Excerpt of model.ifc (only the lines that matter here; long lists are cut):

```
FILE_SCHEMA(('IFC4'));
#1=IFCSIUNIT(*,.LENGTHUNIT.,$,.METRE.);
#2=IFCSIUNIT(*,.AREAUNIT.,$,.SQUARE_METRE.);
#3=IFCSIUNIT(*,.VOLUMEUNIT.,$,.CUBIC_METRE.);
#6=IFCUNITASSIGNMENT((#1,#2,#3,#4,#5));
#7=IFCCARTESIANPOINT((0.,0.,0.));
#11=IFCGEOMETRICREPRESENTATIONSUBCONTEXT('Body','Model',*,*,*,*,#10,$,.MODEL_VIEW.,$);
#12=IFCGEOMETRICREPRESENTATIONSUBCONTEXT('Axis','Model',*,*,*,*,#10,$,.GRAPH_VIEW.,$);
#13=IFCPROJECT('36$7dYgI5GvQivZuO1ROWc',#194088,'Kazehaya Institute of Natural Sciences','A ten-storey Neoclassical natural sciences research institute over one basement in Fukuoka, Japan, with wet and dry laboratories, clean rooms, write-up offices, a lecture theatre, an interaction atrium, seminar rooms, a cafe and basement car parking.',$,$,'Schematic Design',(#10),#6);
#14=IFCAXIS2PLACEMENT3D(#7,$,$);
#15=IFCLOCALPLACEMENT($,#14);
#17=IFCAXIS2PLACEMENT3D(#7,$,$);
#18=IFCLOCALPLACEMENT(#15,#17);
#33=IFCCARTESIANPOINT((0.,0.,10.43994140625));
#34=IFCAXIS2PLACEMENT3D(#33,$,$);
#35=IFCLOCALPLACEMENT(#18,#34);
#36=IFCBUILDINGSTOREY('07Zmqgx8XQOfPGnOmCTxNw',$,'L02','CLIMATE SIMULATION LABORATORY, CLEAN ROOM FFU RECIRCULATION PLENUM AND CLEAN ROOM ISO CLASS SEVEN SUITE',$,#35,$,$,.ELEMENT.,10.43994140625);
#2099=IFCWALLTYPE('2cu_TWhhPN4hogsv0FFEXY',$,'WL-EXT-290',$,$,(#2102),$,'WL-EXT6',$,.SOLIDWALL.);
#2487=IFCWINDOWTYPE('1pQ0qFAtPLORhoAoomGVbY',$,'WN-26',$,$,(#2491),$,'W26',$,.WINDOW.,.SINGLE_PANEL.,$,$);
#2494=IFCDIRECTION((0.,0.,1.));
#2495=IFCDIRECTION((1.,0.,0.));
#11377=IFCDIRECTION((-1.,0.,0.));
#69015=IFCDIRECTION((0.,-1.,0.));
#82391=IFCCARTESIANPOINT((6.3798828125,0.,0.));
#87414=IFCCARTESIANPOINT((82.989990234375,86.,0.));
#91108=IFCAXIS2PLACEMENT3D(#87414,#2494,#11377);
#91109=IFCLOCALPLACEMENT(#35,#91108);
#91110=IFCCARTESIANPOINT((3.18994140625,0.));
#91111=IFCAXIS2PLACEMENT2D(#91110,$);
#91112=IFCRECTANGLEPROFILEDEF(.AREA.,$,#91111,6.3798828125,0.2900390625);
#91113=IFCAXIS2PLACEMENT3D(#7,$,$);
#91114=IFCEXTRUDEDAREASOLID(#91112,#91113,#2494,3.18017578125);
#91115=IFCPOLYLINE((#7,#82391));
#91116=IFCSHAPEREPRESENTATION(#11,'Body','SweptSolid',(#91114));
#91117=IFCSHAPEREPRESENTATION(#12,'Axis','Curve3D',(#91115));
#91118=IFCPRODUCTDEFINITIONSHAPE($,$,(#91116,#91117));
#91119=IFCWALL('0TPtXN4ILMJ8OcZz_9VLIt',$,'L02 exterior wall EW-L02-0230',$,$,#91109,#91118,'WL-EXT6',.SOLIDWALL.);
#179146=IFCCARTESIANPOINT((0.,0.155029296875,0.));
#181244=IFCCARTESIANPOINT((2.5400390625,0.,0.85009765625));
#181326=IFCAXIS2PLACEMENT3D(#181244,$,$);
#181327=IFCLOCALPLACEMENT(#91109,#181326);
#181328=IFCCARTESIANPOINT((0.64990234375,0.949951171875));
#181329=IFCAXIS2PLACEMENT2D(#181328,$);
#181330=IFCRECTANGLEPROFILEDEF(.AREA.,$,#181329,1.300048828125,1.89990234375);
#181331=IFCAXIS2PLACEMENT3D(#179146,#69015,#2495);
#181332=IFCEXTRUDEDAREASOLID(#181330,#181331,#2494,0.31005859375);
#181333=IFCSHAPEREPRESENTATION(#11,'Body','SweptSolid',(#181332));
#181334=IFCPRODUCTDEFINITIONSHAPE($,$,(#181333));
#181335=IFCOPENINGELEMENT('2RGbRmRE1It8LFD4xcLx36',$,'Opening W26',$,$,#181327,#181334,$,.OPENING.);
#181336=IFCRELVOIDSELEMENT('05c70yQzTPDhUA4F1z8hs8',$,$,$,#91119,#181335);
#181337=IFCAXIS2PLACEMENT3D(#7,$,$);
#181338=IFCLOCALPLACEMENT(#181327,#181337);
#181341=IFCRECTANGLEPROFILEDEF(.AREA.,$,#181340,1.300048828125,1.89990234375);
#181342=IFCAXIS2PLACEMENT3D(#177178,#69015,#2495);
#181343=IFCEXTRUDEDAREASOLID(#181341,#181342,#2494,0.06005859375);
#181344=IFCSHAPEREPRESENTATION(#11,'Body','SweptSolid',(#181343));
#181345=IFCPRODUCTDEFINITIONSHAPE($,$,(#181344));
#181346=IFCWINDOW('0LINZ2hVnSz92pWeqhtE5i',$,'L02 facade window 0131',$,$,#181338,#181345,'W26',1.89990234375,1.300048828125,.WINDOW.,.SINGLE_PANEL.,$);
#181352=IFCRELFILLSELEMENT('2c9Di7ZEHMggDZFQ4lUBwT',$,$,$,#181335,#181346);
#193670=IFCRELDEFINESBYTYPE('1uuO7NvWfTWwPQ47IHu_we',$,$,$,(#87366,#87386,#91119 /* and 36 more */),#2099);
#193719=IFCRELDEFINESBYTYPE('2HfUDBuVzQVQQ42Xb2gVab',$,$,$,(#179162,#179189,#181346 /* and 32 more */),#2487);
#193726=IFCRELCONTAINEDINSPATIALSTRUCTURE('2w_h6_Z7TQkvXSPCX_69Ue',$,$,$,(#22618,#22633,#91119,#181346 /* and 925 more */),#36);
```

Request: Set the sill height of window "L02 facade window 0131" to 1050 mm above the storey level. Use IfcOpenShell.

```python
import numpy as np
import ifcopenshell
import ifcopenshell.api.geometry
import ifcopenshell.geom
import ifcopenshell.util.element
import ifcopenshell.util.placement
import ifcopenshell.util.shape
import ifcopenshell.util.unit

model = ifcopenshell.open("model.ifc")
unit_scale = ifcopenshell.util.unit.calculate_unit_scale(model)

window = model.by_id(181346)
opening = window.FillsVoids[0].RelatingOpeningElement
storey = ifcopenshell.util.element.get_container(window, ifc_class="IfcBuildingStorey")
level = ifcopenshell.util.placement.get_local_placement(storey.ObjectPlacement)[2, 3]

# The opening's origin need not be at the sill, so measure its lowest point.
shape = ifcopenshell.geom.create_shape(ifcopenshell.geom.settings(), opening)
bottom = ifcopenshell.util.shape.get_shape_bottom_elevation(shape, shape.geometry) / unit_scale
dz = level + 1.05 / unit_scale - bottom

shift = np.array([0.0, 0.0, dz])
# The window is placed relative to its opening, so it follows when the opening moves.
matrix = ifcopenshell.util.placement.get_local_placement(opening.ObjectPlacement)
matrix[:3, 3] += shift
ifcopenshell.api.geometry.edit_object_placement(
    model, product=opening, matrix=matrix, is_si=False, should_transform_children=True
)

print(f"moved by {dz * unit_scale:+.3f} m")

model.write("model_edited.ifc")
```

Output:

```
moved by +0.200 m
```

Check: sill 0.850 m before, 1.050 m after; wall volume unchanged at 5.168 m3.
